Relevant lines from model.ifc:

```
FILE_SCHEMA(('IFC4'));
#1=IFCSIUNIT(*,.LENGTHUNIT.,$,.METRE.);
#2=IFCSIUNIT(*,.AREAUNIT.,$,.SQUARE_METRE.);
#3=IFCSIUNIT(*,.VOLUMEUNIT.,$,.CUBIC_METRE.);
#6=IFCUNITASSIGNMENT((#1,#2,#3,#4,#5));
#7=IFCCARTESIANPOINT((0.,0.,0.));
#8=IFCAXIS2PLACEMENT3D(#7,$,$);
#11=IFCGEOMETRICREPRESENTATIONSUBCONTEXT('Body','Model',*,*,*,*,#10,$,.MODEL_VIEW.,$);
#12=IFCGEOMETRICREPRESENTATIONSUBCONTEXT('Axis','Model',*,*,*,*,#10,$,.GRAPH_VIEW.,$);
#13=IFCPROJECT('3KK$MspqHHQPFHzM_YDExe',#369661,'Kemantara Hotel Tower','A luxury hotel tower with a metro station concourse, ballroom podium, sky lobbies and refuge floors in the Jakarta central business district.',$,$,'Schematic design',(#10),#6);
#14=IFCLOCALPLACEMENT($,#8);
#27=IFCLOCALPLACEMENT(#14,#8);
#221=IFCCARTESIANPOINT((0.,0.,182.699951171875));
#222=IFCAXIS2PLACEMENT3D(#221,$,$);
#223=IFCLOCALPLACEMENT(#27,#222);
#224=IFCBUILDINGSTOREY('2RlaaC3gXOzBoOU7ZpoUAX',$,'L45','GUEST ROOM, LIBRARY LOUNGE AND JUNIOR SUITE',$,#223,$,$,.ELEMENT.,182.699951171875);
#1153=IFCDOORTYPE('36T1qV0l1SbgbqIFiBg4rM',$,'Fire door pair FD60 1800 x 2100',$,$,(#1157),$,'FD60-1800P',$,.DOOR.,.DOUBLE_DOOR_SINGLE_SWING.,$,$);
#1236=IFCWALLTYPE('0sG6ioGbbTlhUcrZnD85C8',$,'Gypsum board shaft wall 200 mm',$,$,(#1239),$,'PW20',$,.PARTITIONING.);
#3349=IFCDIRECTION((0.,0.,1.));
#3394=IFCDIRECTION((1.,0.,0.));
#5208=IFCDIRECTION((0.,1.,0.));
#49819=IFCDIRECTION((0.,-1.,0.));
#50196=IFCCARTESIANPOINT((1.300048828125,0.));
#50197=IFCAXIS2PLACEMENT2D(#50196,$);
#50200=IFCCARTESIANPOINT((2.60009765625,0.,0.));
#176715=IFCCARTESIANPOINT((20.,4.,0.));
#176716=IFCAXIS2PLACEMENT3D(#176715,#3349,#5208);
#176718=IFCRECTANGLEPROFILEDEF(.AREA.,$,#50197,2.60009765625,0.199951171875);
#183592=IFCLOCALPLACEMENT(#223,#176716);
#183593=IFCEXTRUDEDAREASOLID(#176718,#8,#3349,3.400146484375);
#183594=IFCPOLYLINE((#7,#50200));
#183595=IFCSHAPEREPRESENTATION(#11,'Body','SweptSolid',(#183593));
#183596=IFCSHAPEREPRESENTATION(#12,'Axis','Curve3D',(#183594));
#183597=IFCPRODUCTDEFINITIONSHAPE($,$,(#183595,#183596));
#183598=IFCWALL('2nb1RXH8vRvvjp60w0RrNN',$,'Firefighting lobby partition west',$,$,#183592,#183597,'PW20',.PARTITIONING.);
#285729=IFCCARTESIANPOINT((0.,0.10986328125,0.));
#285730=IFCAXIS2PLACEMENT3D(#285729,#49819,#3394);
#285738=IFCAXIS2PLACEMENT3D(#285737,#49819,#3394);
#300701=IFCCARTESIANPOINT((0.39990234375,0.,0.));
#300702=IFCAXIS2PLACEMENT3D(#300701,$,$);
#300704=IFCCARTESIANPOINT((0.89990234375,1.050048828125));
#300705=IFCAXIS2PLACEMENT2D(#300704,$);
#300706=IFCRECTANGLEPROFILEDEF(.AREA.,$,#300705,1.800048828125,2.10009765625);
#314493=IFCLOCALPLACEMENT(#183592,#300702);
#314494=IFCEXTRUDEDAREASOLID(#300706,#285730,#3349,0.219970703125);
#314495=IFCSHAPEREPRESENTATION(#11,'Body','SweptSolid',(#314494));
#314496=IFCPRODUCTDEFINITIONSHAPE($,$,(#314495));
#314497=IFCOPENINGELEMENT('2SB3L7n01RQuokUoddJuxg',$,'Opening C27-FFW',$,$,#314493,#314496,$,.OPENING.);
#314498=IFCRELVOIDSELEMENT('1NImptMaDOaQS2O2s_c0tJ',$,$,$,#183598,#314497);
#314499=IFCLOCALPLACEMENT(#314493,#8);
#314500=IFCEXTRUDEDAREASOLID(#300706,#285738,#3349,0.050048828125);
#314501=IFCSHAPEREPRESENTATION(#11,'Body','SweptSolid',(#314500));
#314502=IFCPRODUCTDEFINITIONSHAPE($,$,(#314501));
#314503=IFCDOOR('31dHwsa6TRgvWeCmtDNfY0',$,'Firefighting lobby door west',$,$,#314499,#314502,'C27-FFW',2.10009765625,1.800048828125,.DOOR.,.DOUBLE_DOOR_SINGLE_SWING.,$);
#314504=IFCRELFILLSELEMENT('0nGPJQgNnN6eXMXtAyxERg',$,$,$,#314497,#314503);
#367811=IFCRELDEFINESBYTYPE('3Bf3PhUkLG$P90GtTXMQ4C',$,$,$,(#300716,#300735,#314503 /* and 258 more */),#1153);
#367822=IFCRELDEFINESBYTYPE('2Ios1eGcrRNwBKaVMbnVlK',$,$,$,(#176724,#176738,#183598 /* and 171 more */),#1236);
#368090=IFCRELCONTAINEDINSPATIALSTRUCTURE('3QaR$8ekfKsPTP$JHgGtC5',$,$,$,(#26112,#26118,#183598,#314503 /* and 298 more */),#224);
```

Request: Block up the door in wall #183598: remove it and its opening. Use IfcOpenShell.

```python
import ifcopenshell
import ifcopenshell.api.feature
import ifcopenshell.api.root
import ifcopenshell.geom
import ifcopenshell.util.shape

model = ifcopenshell.open("model.ifc")
settings = ifcopenshell.geom.settings()


def volume(element):
    """Net volume in cubic metres, openings subtracted."""
    shape = ifcopenshell.geom.create_shape(settings, element)
    return ifcopenshell.util.shape.get_volume(shape.geometry)


door = model.by_id(314503)
opening = door.FillsVoids[0].RelatingOpeningElement
wall = opening.VoidsElements[0].RelatingBuildingElement
before = volume(wall)

ifcopenshell.api.root.remove_product(model, product=door)
ifcopenshell.api.feature.remove_feature(model, feature=opening)

after = volume(wall)

print(f"wall volume {before:.3f} -> {after:.3f} m3")

model.write("model_updated.ifc")
```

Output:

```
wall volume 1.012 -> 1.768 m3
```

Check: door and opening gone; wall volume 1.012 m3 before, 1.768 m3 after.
